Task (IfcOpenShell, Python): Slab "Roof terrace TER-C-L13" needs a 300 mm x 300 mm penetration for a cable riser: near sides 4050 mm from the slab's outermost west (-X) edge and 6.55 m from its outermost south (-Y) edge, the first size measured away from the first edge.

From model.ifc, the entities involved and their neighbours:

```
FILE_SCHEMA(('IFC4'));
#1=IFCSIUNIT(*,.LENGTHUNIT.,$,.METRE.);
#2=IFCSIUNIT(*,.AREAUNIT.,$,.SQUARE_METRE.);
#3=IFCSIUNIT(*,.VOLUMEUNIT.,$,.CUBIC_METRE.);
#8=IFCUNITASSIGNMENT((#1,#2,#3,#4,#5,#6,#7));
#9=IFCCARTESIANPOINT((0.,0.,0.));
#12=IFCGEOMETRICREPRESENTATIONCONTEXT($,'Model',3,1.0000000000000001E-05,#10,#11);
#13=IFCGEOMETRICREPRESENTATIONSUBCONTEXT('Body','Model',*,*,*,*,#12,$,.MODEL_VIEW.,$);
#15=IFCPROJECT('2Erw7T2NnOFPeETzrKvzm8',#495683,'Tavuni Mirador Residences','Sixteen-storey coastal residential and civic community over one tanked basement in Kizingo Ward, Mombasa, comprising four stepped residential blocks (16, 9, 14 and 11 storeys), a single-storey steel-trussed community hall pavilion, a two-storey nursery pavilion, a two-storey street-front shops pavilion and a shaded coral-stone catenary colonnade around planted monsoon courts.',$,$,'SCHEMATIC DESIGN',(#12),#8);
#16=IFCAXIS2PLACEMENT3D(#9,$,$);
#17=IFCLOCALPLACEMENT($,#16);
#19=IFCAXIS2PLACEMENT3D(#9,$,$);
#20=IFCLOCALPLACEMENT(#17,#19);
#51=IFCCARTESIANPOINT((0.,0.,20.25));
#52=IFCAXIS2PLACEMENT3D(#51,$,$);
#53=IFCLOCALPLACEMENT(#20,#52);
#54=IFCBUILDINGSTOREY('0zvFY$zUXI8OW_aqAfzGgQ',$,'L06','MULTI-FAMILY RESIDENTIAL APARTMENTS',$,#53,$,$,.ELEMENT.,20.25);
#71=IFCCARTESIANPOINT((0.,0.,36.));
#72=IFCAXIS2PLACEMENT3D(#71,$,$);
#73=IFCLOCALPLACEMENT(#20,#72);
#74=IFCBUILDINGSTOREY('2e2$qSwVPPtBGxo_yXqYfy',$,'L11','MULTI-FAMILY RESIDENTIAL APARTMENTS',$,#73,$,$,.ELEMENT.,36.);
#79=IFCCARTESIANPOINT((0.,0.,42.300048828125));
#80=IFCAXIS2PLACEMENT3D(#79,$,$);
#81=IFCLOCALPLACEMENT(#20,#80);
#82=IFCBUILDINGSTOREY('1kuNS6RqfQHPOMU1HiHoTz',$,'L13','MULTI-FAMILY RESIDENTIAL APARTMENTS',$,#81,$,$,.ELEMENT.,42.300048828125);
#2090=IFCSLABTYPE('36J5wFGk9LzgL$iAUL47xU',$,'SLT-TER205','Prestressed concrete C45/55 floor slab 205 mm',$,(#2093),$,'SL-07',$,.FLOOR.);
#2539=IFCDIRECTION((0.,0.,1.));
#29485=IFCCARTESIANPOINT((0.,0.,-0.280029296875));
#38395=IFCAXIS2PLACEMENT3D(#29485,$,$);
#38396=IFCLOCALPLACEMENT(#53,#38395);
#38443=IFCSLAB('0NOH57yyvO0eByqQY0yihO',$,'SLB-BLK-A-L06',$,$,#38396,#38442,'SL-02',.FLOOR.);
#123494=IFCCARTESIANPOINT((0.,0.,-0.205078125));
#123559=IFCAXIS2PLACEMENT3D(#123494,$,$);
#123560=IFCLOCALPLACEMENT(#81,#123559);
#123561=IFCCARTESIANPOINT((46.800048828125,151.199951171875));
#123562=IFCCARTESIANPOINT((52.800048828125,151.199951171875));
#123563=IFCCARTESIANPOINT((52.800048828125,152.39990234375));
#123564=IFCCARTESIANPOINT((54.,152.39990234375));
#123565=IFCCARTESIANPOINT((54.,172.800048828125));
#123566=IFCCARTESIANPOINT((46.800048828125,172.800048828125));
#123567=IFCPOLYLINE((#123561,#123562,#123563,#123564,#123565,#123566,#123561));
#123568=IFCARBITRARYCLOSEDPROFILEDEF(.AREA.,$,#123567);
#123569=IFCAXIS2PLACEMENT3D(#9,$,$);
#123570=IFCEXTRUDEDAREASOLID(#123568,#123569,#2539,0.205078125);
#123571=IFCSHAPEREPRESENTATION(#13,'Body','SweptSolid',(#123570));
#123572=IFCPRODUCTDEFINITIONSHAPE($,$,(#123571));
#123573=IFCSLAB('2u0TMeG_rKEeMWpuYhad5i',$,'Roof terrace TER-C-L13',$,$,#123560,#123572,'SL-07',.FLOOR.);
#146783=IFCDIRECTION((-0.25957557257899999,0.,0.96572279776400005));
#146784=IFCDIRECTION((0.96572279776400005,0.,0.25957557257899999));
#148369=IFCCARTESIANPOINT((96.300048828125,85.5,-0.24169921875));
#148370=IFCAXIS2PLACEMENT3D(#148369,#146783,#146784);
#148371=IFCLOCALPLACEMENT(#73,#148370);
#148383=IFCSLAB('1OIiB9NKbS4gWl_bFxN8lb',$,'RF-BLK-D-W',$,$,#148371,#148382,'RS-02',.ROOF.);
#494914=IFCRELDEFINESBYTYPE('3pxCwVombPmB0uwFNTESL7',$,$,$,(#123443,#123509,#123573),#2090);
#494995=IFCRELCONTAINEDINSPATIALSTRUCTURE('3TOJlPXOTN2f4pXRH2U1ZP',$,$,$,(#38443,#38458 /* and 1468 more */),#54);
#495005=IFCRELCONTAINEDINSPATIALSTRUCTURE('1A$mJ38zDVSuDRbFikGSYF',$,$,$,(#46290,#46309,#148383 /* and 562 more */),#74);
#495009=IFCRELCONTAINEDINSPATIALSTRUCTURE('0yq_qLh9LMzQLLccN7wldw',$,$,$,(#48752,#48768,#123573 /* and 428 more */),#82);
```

```python
import numpy as np
import ifcopenshell
import ifcopenshell.api.feature
import ifcopenshell.api.geometry
import ifcopenshell.api.root
import ifcopenshell.geom
import ifcopenshell.util.placement
import ifcopenshell.util.representation
import ifcopenshell.util.shape
import ifcopenshell.util.unit

model = ifcopenshell.open("model.ifc")
unit_scale = ifcopenshell.util.unit.calculate_unit_scale(model)
settings = ifcopenshell.geom.settings()


def volume(element):
    """Net volume in cubic metres, openings subtracted."""
    shape = ifcopenshell.geom.create_shape(settings, element)
    return ifcopenshell.util.shape.get_volume(shape.geometry)


slab = model.by_guid("2u0TMeG_rKEeMWpuYhad5i")
before = volume(slab)

# Extent in the slab's own axes, in metres. The edges named are its -X and -Y sides.
slab_shape = ifcopenshell.geom.create_shape(settings, slab)
vertices = ifcopenshell.util.shape.get_vertices(slab_shape.geometry)
x_min, y_min, bottom = vertices.min(axis=0)
top = vertices[:, 2].max()

opening = ifcopenshell.api.root.create_entity(model, ifc_class="IfcOpeningElement", name="Cable riser opening", predefined_type="OPENING")
context = ifcopenshell.util.representation.get_context(model, "Model", "Body", "MODEL_VIEW")
width, depth = 0.3, 0.3
outline = [(0.0, 0.0), (width, 0.0), (width, depth), (0.0, depth), (0.0, 0.0)]
# Overshoot both faces by 50 mm so the cut is clean.
shape = ifcopenshell.api.geometry.add_slab_representation(
    model, context=context, depth=top - bottom + 0.1, polyline=outline
)
ifcopenshell.api.geometry.assign_representation(model, product=opening, representation=shape)

matrix = ifcopenshell.util.placement.get_local_placement(slab.ObjectPlacement)
matrix[:, 3] = matrix @ np.append(np.array([x_min + 4.05, y_min + 6.55, bottom - 0.05]) / unit_scale, 1.0)
ifcopenshell.api.geometry.edit_object_placement(model, product=opening, matrix=matrix, is_si=False)
ifcopenshell.api.feature.add_feature(model, feature=opening, element=slab)

after = volume(slab)

print(f"slab volume {before:.3f} -> {after:.3f} m3")

model.write("model_updated.ifc")
```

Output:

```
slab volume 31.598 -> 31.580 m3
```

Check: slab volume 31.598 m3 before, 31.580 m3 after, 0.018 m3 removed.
